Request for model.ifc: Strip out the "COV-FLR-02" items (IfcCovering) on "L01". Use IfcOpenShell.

First a look at what the model holds.

```python
import ifcopenshell
import ifcopenshell.util.element

model = ifcopenshell.open("model.ifc")
print(model.schema)
storey = next(s for s in model.by_type("IfcBuildingStorey") if s.Name == "L01")
coverings = [e for e in ifcopenshell.util.element.get_decomposition(storey) if e.is_a("IfcCovering")]
seen = {}
for e in coverings:
    element_type = ifcopenshell.util.element.get_type(e)
    name = element_type.Name if element_type not in (None, e) else None
    seen[name] = seen.get(name, 0) + 1
for name, count in sorted(seen.items(), key=str):
    print(count, "x", name)
```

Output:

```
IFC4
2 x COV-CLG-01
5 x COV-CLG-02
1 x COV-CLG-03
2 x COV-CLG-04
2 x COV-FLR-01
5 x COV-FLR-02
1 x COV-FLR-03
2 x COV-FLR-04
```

```python
import ifcopenshell
import ifcopenshell.api.root
import ifcopenshell.util.element

model = ifcopenshell.open("model.ifc")

storey = next(s for s in model.by_type("IfcBuildingStorey") if s.Name == "L01")
coverings = [e for e in ifcopenshell.util.element.get_decomposition(storey) if e.is_a("IfcCovering")]
targets = [e for e in coverings if (t := ifcopenshell.util.element.get_type(e)) not in (None, e) and t.Name == "COV-FLR-02"]

for e in targets:
    ifcopenshell.api.root.remove_product(model, product=e)
print(len(targets), "removed")

model.write("model_rev.ifc")
```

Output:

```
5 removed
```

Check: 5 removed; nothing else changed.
